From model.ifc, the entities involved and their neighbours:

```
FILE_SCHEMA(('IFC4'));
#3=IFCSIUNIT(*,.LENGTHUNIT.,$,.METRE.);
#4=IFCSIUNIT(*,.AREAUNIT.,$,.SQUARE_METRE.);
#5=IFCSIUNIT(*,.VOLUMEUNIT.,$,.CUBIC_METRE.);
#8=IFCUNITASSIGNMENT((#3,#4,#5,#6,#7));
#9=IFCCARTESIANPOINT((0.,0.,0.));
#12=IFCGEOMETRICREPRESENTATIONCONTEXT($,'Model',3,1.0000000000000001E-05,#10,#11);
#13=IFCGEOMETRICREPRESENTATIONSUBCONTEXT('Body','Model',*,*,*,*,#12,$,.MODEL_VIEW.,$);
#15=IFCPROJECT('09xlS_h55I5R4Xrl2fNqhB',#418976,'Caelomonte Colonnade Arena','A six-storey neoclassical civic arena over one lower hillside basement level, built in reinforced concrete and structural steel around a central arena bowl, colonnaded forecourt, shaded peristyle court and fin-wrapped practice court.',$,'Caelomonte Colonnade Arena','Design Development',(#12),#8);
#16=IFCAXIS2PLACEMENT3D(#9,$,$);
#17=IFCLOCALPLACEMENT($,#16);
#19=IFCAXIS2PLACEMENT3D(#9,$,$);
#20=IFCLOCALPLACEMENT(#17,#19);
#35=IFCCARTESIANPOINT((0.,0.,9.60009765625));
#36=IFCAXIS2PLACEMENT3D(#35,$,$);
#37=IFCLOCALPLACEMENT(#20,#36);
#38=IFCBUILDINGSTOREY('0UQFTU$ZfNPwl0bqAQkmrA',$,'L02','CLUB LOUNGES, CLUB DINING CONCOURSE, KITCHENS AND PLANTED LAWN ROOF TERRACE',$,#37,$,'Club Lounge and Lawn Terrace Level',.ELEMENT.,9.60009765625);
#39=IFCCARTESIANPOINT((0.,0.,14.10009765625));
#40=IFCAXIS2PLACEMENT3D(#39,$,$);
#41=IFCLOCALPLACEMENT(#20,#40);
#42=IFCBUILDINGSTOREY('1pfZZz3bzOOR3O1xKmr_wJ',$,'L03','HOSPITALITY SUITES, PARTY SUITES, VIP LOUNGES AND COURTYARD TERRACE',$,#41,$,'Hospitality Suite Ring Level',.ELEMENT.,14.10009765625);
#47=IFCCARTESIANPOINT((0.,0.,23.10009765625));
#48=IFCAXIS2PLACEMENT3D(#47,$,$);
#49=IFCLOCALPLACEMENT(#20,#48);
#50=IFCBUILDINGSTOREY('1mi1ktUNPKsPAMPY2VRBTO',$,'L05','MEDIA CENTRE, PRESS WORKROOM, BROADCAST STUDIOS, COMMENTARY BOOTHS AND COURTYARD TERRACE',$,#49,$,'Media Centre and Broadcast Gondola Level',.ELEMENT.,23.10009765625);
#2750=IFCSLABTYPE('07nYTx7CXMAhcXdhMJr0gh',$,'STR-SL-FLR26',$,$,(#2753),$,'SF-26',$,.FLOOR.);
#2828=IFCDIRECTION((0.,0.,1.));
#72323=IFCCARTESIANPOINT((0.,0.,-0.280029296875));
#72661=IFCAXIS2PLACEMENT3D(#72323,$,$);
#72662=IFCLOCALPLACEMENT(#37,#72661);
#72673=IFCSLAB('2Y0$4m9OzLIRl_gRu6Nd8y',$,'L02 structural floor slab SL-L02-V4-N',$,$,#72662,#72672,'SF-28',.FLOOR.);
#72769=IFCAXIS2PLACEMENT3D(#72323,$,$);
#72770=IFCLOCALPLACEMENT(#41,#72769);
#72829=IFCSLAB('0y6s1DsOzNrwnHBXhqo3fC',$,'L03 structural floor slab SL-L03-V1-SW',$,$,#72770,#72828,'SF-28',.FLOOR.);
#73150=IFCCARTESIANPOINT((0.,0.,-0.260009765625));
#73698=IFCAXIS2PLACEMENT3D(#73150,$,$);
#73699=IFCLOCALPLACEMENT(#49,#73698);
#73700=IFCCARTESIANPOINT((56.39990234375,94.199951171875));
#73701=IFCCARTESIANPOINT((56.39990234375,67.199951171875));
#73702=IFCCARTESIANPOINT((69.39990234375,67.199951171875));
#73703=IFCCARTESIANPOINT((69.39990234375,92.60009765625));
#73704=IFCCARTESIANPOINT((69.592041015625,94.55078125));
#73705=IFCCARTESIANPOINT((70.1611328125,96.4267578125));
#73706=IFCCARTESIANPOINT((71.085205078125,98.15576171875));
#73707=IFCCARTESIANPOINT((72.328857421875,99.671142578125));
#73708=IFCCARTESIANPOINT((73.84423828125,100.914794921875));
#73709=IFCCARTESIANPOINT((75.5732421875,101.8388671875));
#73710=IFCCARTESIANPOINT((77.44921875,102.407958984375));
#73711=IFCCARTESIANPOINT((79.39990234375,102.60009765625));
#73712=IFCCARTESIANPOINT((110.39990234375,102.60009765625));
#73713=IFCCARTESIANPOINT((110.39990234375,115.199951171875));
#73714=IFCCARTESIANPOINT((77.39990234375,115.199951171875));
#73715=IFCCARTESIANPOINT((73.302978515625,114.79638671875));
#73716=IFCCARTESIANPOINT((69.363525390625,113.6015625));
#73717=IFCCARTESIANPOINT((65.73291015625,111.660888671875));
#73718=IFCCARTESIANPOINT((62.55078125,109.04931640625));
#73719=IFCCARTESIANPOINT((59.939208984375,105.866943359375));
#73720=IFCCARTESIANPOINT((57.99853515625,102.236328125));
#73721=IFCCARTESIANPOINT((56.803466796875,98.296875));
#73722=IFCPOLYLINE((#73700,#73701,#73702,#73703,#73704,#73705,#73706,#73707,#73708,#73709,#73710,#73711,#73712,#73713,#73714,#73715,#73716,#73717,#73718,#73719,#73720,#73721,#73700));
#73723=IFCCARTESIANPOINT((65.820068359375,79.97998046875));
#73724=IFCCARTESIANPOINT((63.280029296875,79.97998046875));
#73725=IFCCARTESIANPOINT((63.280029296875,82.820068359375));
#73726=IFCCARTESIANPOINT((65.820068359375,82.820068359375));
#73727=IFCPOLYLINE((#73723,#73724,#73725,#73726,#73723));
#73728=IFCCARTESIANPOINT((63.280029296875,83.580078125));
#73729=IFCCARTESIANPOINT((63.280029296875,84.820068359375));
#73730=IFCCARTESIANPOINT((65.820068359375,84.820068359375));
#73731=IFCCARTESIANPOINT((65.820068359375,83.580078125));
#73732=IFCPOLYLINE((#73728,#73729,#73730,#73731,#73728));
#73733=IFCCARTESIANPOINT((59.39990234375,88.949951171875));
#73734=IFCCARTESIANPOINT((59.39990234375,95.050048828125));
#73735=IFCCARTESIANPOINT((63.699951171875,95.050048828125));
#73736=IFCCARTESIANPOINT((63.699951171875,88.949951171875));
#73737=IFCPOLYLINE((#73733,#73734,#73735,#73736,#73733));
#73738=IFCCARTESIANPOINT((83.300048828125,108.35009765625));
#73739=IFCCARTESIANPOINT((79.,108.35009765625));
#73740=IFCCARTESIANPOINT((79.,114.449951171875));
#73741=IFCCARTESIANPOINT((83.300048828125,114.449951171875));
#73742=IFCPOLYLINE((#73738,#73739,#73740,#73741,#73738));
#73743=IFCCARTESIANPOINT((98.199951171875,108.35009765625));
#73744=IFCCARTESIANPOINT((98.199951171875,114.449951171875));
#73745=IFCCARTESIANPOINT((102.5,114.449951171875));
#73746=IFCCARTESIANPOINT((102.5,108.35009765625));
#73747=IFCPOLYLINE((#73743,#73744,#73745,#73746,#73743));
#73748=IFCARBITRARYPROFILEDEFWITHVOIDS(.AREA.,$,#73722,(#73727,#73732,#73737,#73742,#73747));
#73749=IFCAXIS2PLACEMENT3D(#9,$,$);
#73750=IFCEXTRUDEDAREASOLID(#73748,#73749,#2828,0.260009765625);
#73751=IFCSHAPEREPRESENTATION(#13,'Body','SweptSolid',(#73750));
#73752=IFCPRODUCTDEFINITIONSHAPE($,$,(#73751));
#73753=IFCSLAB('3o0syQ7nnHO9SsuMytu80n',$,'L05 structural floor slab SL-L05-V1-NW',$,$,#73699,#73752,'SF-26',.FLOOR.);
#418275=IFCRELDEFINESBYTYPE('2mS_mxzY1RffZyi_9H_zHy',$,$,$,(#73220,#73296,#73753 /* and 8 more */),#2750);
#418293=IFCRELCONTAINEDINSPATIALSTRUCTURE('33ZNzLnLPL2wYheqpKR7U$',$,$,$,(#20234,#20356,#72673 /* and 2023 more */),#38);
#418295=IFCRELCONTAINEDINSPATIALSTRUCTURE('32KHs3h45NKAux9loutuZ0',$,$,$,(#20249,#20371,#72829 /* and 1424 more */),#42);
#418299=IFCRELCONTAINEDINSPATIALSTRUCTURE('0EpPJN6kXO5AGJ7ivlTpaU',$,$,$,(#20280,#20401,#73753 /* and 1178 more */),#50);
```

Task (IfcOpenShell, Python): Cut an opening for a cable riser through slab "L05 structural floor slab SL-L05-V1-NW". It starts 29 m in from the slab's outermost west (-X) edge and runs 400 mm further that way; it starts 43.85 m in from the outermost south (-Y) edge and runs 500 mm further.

```python
import numpy as np
import ifcopenshell
import ifcopenshell.api.feature
import ifcopenshell.api.geometry
import ifcopenshell.api.root
import ifcopenshell.geom
import ifcopenshell.util.placement
import ifcopenshell.util.representation
import ifcopenshell.util.shape
import ifcopenshell.util.unit

model = ifcopenshell.open("model.ifc")
unit_scale = ifcopenshell.util.unit.calculate_unit_scale(model)
settings = ifcopenshell.geom.settings()


def volume(element):
    """Net volume in cubic metres, openings subtracted."""
    shape = ifcopenshell.geom.create_shape(settings, element)
    return ifcopenshell.util.shape.get_volume(shape.geometry)


slab = model.by_id(73753)
before = volume(slab)

# Extent in the slab's own axes, in metres. The edges named are its -X and -Y sides.
slab_shape = ifcopenshell.geom.create_shape(settings, slab)
vertices = ifcopenshell.util.shape.get_vertices(slab_shape.geometry)
x_min, y_min, bottom = vertices.min(axis=0)
top = vertices[:, 2].max()

opening = ifcopenshell.api.root.create_entity(model, ifc_class="IfcOpeningElement", name="Cable riser opening", predefined_type="OPENING")
context = ifcopenshell.util.representation.get_context(model, "Model", "Body", "MODEL_VIEW")
width, depth = 0.4, 0.5
outline = [(0.0, 0.0), (width, 0.0), (width, depth), (0.0, depth), (0.0, 0.0)]
# Overshoot both faces by 50 mm so the cut is clean.
shape = ifcopenshell.api.geometry.add_slab_representation(
    model, context=context, depth=top - bottom + 0.1, polyline=outline
)
ifcopenshell.api.geometry.assign_representation(model, product=opening, representation=shape)

matrix = ifcopenshell.util.placement.get_local_placement(slab.ObjectPlacement)
matrix[:, 3] = matrix @ np.append(np.array([x_min + 29, y_min + 43.85, bottom - 0.05]) / unit_scale, 1.0)
ifcopenshell.api.geometry.edit_object_placement(model, product=opening, matrix=matrix, is_si=False)
ifcopenshell.api.feature.add_feature(model, feature=opening, element=slab)

after = volume(slab)

print(f"slab volume {before:.3f} -> {after:.3f} m3")

model.write("model-out.ifc")
```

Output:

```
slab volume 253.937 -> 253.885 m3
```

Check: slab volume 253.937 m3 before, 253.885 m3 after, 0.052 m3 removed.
